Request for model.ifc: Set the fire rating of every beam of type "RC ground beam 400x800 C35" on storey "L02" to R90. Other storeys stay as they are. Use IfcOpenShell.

First a look at what the model holds.

```python
import ifcopenshell
import ifcopenshell.util.element

model = ifcopenshell.open("model.ifc")
print(model.schema)
storey = next(s for s in model.by_type("IfcBuildingStorey") if s.Name == "L02")
beams = [e for e in ifcopenshell.util.element.get_decomposition(storey) if e.is_a("IfcBeam")]
seen = {}
for e in beams:
    element_type = ifcopenshell.util.element.get_type(e)
    key = (element_type.Name if element_type != e and element_type else None, ifcopenshell.util.element.get_pset(e, "Pset_BeamCommon", "FireRating"))
    seen[key] = seen.get(key, 0) + 1
for (name, value), count in sorted(seen.items(), key=str):
    print(count, "x", name, "|", value)
```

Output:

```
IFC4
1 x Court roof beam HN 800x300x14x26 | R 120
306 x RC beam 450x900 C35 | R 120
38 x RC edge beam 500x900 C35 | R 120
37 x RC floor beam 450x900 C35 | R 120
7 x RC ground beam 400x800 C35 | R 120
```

```python
import ifcopenshell
import ifcopenshell.api.pset
import ifcopenshell.util.element

model = ifcopenshell.open("model.ifc")

storey = next(s for s in model.by_type("IfcBuildingStorey") if s.Name == "L02")
beams = [e for e in ifcopenshell.util.element.get_decomposition(storey) if e.is_a("IfcBeam")]

count = 0
for e in beams:
    element_type = ifcopenshell.util.element.get_type(e)
    if element_type in (None, e) or element_type.Name != "RC ground beam 400x800 C35":
        continue
    # add_pset returns the element's existing set when there is one.
    pset = ifcopenshell.api.pset.add_pset(model, product=e, name="Pset_BeamCommon")
    ifcopenshell.api.pset.edit_pset(model, pset=pset, properties={"FireRating": "R90"})
    count += 1

print(count, "beams updated")

model.write("model-out.ifc")
```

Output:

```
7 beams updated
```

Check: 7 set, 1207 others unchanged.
